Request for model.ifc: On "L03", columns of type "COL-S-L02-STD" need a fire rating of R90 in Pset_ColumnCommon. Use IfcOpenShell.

First a look at what the model holds.

```python
import ifcopenshell
import ifcopenshell.util.element

model = ifcopenshell.open("model.ifc")
print(model.schema)
storey = next(s for s in model.by_type("IfcBuildingStorey") if s.Name == "L03")
columns = [e for e in ifcopenshell.util.element.get_decomposition(storey) if e.is_a("IfcColumn")]
seen = {}
for e in columns:
    element_type = ifcopenshell.util.element.get_type(e)
    key = (element_type.Name if element_type != e and element_type else None, ifcopenshell.util.element.get_pset(e, "Pset_ColumnCommon", "FireRating"))
    seen[key] = seen.get(key, 0) + 1
for (name, value), count in sorted(seen.items(), key=str):
    print(count, "x", name, "|", value)
```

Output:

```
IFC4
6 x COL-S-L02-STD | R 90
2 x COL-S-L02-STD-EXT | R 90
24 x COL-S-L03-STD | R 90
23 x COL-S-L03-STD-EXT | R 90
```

```python
import ifcopenshell
import ifcopenshell.api.pset
import ifcopenshell.util.element

model = ifcopenshell.open("model.ifc")

storey = next(s for s in model.by_type("IfcBuildingStorey") if s.Name == "L03")
columns = [e for e in ifcopenshell.util.element.get_decomposition(storey) if e.is_a("IfcColumn")]

count = 0
for e in columns:
    element_type = ifcopenshell.util.element.get_type(e)
    if element_type in (None, e) or element_type.Name != "COL-S-L02-STD":
        continue
    # add_pset returns the element's existing set when there is one.
    pset = ifcopenshell.api.pset.add_pset(model, product=e, name="Pset_ColumnCommon")
    ifcopenshell.api.pset.edit_pset(model, pset=pset, properties={"FireRating": "R90"})
    count += 1

print(count, "columns updated")

model.write("model_edited.ifc")
```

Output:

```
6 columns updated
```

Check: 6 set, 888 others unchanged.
